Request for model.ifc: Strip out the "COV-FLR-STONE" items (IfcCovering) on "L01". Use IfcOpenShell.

First a look at what the model holds.

```python
import ifcopenshell
import ifcopenshell.util.element

model = ifcopenshell.open("model.ifc")
print(model.schema)
storey = next(s for s in model.by_type("IfcBuildingStorey") if s.Name == "L01")
coverings = [e for e in ifcopenshell.util.element.get_decomposition(storey) if e.is_a("IfcCovering")]
seen = {}
for e in coverings:
    element_type = ifcopenshell.util.element.get_type(e)
    name = element_type.Name if element_type not in (None, e) else None
    seen[name] = seen.get(name, 0) + 1
for name, count in sorted(seen.items(), key=str):
    print(count, "x", name)
```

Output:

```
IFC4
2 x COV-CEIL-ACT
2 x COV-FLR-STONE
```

```python
import ifcopenshell
import ifcopenshell.api.root
import ifcopenshell.util.element

model = ifcopenshell.open("model.ifc")

storey = next(s for s in model.by_type("IfcBuildingStorey") if s.Name == "L01")
coverings = [e for e in ifcopenshell.util.element.get_decomposition(storey) if e.is_a("IfcCovering")]
targets = [e for e in coverings if (t := ifcopenshell.util.element.get_type(e)) not in (None, e) and t.Name == "COV-FLR-STONE"]

for e in targets:
    ifcopenshell.api.root.remove_product(model, product=e)
print(len(targets), "removed")

model.write("model_rev.ifc")
```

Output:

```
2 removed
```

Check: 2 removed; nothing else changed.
